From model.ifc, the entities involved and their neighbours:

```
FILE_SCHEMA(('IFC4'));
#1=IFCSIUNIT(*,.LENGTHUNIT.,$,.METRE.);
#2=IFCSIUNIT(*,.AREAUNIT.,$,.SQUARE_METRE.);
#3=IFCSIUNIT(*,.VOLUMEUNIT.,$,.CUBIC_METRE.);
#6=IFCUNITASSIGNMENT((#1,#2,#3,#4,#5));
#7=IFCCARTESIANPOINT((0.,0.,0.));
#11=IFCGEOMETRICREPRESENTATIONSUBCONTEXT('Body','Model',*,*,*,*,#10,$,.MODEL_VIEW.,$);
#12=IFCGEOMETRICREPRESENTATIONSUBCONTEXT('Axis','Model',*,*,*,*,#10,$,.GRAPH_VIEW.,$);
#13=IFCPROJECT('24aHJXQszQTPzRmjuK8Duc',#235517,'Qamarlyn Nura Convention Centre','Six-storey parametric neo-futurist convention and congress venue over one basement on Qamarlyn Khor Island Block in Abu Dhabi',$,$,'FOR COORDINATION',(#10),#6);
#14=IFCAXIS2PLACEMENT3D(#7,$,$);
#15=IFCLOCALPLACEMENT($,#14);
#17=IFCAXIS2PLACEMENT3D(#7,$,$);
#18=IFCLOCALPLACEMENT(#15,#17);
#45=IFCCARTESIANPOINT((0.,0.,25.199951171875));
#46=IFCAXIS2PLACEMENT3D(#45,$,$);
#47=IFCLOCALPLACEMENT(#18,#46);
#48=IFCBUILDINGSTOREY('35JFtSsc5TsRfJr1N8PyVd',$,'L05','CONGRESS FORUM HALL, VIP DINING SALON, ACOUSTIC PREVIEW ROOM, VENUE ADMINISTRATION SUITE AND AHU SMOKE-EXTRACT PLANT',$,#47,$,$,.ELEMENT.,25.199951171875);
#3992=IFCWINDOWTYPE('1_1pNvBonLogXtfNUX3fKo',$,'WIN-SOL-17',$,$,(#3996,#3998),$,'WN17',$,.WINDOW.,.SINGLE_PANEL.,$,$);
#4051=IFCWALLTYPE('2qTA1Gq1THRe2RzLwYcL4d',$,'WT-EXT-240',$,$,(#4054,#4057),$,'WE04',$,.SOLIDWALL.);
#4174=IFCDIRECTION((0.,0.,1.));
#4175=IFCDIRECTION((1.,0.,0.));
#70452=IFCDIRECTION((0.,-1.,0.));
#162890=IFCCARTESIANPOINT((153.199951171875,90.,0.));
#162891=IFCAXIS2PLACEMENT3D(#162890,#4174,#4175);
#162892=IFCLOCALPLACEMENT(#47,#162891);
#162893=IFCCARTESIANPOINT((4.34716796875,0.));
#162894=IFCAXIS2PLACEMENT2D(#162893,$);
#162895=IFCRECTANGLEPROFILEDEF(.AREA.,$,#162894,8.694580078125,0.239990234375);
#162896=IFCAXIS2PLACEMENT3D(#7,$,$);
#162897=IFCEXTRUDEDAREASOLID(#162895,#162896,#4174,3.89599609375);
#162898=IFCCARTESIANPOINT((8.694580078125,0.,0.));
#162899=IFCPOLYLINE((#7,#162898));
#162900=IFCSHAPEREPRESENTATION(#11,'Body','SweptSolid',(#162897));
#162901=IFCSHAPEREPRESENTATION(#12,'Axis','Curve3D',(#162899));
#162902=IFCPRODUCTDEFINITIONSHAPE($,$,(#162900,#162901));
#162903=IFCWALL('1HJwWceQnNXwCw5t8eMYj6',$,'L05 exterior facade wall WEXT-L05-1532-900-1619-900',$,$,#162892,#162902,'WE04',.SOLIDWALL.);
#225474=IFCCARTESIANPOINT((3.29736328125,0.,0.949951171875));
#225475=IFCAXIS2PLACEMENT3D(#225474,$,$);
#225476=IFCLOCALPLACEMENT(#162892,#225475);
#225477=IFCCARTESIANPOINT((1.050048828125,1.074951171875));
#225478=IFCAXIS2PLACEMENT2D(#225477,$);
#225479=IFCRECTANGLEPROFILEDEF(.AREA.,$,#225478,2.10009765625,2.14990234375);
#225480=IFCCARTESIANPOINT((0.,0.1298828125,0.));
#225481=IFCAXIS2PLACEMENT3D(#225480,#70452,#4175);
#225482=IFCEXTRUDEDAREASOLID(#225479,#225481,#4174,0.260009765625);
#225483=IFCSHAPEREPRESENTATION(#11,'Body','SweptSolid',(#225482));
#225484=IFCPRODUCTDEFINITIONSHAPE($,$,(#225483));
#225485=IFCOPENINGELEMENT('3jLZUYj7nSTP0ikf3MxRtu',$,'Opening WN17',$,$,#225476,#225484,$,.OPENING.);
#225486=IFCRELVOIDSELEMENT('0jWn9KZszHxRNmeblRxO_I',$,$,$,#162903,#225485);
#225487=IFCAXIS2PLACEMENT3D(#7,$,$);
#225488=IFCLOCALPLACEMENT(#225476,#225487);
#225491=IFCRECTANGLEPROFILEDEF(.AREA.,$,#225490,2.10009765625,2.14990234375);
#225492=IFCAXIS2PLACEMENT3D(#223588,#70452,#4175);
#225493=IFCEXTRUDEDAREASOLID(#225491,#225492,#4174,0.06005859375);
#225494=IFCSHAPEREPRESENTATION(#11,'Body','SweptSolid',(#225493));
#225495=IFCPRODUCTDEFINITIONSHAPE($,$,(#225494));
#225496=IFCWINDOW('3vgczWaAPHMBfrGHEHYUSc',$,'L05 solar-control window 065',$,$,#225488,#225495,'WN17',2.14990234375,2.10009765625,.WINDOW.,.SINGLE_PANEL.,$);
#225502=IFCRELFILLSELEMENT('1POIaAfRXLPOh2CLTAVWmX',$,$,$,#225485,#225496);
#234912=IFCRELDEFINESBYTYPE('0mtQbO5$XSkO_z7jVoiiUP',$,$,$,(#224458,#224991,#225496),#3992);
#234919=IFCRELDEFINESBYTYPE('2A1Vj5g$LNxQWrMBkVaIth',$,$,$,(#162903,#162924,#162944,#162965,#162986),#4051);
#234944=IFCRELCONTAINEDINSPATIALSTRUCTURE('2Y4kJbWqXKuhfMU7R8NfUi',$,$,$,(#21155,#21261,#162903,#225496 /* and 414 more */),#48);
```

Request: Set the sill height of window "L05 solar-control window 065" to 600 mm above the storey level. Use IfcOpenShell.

```python
import numpy as np
import ifcopenshell
import ifcopenshell.api.geometry
import ifcopenshell.geom
import ifcopenshell.util.element
import ifcopenshell.util.placement
import ifcopenshell.util.shape
import ifcopenshell.util.unit

model = ifcopenshell.open("model.ifc")
unit_scale = ifcopenshell.util.unit.calculate_unit_scale(model)

window = model.by_guid("3vgczWaAPHMBfrGHEHYUSc")
opening = window.FillsVoids[0].RelatingOpeningElement
storey = ifcopenshell.util.element.get_container(window, ifc_class="IfcBuildingStorey")
level = ifcopenshell.util.placement.get_local_placement(storey.ObjectPlacement)[2, 3]

# The opening's origin need not be at the sill, so measure its lowest point.
shape = ifcopenshell.geom.create_shape(ifcopenshell.geom.settings(), opening)
bottom = ifcopenshell.util.shape.get_shape_bottom_elevation(shape, shape.geometry) / unit_scale
dz = level + 0.6 - bottom

shift = np.array([0.0, 0.0, dz])
# The window is placed relative to its opening, so it follows when the opening moves.
matrix = ifcopenshell.util.placement.get_local_placement(opening.ObjectPlacement)
matrix[:3, 3] += shift
ifcopenshell.api.geometry.edit_object_placement(
    model, product=opening, matrix=matrix, is_si=False, should_transform_children=True
)

print(f"moved by {dz * unit_scale:+.3f} m")

model.write("model_edited.ifc")
```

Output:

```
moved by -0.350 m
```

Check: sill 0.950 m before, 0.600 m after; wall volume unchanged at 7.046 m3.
